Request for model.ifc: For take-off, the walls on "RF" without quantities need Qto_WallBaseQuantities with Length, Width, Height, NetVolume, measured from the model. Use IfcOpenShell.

First a look at what the model holds.

```python
import ifcopenshell
import ifcopenshell.util.element
import ifcopenshell.util.unit

model = ifcopenshell.open("model.ifc")
print(model.schema)
for unit_type in ("LENGTHUNIT", "AREAUNIT", "VOLUMEUNIT"):
    print(unit_type, ifcopenshell.util.unit.calculate_unit_scale(model, unit_type))
storey = next(s for s in model.by_type("IfcBuildingStorey") if s.Name == "RF")
walls = [e for e in ifcopenshell.util.element.get_decomposition(storey) if e.is_a("IfcWall")]
for e in sorted(walls, key=lambda e: e.id()):
    print(e.id(), e.is_a(), e.Name, list(ifcopenshell.util.element.get_psets(e, qtos_only=True)), sep=" | ")
```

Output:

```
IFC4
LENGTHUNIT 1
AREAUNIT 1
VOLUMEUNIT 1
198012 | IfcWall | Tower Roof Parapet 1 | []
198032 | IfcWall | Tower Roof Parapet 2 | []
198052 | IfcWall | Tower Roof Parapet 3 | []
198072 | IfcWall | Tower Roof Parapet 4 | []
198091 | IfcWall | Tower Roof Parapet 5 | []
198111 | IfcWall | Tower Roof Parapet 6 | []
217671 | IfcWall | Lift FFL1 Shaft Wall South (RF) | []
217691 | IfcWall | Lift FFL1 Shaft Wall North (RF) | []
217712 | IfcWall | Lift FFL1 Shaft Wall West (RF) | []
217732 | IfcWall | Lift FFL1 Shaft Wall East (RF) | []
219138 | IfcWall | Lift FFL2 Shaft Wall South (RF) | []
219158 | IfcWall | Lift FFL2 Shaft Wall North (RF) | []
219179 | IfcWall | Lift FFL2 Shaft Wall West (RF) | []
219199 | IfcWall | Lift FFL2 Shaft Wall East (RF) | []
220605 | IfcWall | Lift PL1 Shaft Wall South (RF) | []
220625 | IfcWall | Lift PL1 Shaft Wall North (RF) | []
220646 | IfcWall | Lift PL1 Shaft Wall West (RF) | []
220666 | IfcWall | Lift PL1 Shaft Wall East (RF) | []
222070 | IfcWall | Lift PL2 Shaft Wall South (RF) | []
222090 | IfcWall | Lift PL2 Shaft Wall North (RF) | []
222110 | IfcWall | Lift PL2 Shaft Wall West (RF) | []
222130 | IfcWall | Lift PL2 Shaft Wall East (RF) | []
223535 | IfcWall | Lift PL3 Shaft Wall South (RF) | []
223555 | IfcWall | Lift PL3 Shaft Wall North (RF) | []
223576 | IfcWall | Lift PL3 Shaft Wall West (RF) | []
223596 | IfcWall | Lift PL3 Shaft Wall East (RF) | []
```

```python
import ifcopenshell
import ifcopenshell.api.pset
import ifcopenshell.geom
import ifcopenshell.util.element
import ifcopenshell.util.shape
import ifcopenshell.util.unit

model = ifcopenshell.open("model.ifc")
unit_scale = ifcopenshell.util.unit.calculate_unit_scale(model)
volume_scale = ifcopenshell.util.unit.calculate_unit_scale(model, "VOLUMEUNIT")
settings = ifcopenshell.geom.settings()

storey = next(s for s in model.by_type("IfcBuildingStorey") if s.Name == "RF")
walls = [e for e in ifcopenshell.util.element.get_decomposition(storey) if e.is_a("IfcWall")]

for e in sorted(walls, key=lambda e: e.id()):
    if ifcopenshell.util.element.get_psets(e, qtos_only=True, should_inherit=False):
        continue
    # Geometry comes back in metres, in the element's own axes.
    shape = ifcopenshell.geom.create_shape(settings, e)
    values = {
        "Length": ifcopenshell.util.shape.get_x(shape.geometry) / unit_scale,
        "Width": ifcopenshell.util.shape.get_y(shape.geometry) / unit_scale,
        "Height": ifcopenshell.util.shape.get_z(shape.geometry) / unit_scale,
        "NetVolume": ifcopenshell.util.shape.get_volume(shape.geometry) / volume_scale,
    }
    qto = ifcopenshell.api.pset.add_qto(model, product=e, name="Qto_WallBaseQuantities")
    ifcopenshell.api.pset.edit_qto(model, qto=qto, properties=values)
    print(e.id(), {k: round(v, 3) for k, v in values.items()})

model.write("model_rev.ifc")
```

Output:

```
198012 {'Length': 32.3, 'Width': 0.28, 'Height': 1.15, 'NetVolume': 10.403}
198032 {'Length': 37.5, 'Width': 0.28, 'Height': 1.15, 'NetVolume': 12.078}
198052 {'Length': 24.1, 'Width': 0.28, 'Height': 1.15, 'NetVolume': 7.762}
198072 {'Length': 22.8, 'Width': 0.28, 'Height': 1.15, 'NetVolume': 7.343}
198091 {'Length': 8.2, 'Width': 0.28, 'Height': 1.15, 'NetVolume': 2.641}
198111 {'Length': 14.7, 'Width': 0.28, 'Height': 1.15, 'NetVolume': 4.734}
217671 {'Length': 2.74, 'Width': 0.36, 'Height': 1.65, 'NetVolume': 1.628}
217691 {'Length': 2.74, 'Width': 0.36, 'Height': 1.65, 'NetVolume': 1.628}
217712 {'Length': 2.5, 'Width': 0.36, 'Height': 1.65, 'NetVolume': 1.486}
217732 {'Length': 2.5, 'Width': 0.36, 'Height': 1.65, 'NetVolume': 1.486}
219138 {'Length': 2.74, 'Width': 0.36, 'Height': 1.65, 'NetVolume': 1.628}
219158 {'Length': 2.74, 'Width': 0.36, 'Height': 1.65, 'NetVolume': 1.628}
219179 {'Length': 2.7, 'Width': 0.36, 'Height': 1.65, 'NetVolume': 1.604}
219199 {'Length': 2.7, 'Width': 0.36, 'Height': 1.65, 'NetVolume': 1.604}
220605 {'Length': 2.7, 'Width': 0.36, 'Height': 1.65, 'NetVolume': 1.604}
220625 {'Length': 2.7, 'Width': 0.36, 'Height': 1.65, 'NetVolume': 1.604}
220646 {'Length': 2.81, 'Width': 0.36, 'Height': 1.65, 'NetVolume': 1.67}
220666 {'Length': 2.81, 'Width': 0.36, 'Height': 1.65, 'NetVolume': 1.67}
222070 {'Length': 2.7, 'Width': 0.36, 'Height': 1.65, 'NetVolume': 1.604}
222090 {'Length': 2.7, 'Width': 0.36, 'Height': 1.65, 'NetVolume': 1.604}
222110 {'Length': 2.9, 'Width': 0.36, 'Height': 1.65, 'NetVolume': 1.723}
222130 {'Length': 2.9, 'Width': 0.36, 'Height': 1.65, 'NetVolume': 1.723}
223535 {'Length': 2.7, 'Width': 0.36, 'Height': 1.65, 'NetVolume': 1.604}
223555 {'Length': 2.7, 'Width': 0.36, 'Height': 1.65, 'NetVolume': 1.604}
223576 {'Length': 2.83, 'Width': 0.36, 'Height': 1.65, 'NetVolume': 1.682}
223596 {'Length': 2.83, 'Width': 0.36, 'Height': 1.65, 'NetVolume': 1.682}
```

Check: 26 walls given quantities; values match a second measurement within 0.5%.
